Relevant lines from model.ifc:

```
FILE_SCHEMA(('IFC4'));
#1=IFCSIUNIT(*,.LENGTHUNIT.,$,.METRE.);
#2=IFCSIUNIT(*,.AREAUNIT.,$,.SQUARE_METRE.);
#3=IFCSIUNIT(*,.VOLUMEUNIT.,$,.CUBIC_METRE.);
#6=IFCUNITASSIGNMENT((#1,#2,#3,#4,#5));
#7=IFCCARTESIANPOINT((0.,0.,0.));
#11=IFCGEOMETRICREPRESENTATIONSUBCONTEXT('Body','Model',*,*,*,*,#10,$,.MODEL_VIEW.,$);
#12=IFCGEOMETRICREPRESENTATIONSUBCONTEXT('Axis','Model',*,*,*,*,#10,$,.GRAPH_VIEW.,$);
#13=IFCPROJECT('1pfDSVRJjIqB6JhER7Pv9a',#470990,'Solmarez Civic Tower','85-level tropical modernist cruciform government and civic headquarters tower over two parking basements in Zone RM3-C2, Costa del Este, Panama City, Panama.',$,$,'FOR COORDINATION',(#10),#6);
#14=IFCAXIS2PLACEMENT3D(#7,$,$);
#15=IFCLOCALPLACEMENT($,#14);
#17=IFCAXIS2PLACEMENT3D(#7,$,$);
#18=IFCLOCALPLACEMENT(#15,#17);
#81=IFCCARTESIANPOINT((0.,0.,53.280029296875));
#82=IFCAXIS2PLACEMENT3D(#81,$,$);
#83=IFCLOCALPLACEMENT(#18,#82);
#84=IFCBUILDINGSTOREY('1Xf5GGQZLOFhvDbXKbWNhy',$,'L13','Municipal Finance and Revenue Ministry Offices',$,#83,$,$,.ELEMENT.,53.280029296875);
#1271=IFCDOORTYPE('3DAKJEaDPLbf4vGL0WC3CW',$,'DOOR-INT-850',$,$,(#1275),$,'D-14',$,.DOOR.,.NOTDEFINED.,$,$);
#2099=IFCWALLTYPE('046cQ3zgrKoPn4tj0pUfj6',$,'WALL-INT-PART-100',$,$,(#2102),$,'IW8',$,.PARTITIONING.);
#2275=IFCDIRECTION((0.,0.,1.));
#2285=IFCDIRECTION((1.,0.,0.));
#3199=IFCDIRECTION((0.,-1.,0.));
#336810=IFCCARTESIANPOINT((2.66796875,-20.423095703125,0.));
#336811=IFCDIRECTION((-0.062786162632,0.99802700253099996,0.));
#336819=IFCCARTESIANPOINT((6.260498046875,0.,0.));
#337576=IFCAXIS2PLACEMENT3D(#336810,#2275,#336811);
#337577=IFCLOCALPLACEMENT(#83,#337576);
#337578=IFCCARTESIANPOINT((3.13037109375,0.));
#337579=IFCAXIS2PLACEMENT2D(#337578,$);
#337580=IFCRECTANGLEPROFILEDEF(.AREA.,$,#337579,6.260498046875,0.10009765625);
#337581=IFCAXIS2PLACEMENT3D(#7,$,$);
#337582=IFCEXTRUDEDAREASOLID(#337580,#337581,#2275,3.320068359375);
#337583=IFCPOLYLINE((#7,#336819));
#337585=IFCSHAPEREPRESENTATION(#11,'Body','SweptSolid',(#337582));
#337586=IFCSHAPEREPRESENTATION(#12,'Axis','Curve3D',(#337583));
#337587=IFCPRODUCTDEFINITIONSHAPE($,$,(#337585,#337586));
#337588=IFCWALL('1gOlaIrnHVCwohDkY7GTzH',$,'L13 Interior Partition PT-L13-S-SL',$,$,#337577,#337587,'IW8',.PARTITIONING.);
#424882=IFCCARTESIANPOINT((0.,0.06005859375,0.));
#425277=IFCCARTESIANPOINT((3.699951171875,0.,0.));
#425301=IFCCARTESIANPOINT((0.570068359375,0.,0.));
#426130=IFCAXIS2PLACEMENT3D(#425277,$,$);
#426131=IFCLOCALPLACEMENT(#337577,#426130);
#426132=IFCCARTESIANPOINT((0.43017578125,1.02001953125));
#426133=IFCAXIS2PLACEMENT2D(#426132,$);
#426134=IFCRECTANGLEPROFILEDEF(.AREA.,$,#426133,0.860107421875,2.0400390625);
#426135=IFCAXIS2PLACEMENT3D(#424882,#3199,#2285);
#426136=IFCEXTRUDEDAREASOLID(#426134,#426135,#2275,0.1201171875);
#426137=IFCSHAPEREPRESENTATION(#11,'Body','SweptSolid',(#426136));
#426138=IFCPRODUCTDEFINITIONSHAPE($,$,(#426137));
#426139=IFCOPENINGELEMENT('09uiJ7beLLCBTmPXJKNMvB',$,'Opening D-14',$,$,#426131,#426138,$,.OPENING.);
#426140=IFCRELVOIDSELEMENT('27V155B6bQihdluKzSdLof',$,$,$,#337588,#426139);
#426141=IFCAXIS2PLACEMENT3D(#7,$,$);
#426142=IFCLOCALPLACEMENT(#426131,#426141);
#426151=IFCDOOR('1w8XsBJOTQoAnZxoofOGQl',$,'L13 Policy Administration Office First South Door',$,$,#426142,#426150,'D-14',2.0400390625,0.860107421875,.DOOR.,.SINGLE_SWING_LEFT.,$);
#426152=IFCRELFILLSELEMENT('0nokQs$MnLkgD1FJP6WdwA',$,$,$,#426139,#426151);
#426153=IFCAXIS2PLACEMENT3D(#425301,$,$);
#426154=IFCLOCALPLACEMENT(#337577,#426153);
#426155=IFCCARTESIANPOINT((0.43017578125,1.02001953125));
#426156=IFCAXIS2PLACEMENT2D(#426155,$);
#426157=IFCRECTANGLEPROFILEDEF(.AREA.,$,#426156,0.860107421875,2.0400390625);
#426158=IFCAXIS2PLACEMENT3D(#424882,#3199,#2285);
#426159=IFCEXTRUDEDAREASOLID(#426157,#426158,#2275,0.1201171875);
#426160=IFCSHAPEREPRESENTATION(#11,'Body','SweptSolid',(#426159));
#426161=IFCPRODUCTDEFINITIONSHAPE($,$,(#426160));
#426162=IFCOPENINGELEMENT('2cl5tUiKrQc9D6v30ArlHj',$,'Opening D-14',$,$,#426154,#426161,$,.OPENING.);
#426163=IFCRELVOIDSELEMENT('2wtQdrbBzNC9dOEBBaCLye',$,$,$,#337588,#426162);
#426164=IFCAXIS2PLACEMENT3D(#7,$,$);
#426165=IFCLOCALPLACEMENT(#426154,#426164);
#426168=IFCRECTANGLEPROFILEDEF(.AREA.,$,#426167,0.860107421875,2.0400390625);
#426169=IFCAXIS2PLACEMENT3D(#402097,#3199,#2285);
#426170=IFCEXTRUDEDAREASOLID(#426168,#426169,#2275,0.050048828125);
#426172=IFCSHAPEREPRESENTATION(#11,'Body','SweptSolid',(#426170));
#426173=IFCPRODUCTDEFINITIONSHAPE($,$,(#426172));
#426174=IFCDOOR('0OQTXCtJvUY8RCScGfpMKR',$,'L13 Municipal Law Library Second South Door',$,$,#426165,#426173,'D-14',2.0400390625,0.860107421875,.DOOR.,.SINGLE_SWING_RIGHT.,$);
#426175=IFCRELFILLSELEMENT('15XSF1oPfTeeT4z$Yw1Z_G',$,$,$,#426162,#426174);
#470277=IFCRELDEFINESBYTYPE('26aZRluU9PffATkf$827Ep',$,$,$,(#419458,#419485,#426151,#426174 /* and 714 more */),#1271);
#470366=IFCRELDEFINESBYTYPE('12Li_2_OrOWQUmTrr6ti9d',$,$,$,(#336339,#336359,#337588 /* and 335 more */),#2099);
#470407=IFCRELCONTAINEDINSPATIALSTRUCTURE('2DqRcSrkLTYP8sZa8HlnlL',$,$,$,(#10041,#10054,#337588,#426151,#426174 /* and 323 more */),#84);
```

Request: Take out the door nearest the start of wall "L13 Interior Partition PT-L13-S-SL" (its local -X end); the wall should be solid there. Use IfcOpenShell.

```python
import ifcopenshell
import ifcopenshell.api.feature
import ifcopenshell.api.root
import ifcopenshell.geom
import ifcopenshell.util.shape

model = ifcopenshell.open("model.ifc")
settings = ifcopenshell.geom.settings()


def volume(element):
    """Net volume in cubic metres, openings subtracted."""
    shape = ifcopenshell.geom.create_shape(settings, element)
    return ifcopenshell.util.shape.get_volume(shape.geometry)


door = model.by_guid("0OQTXCtJvUY8RCScGfpMKR")
opening = door.FillsVoids[0].RelatingOpeningElement
wall = opening.VoidsElements[0].RelatingBuildingElement
before = volume(wall)

ifcopenshell.api.root.remove_product(model, product=door)
ifcopenshell.api.feature.remove_feature(model, feature=opening)

after = volume(wall)

print(f"wall volume {before:.3f} -> {after:.3f} m3")

model.write("model_v2.ifc")
```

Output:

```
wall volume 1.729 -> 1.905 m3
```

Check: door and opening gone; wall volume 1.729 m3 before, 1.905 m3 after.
